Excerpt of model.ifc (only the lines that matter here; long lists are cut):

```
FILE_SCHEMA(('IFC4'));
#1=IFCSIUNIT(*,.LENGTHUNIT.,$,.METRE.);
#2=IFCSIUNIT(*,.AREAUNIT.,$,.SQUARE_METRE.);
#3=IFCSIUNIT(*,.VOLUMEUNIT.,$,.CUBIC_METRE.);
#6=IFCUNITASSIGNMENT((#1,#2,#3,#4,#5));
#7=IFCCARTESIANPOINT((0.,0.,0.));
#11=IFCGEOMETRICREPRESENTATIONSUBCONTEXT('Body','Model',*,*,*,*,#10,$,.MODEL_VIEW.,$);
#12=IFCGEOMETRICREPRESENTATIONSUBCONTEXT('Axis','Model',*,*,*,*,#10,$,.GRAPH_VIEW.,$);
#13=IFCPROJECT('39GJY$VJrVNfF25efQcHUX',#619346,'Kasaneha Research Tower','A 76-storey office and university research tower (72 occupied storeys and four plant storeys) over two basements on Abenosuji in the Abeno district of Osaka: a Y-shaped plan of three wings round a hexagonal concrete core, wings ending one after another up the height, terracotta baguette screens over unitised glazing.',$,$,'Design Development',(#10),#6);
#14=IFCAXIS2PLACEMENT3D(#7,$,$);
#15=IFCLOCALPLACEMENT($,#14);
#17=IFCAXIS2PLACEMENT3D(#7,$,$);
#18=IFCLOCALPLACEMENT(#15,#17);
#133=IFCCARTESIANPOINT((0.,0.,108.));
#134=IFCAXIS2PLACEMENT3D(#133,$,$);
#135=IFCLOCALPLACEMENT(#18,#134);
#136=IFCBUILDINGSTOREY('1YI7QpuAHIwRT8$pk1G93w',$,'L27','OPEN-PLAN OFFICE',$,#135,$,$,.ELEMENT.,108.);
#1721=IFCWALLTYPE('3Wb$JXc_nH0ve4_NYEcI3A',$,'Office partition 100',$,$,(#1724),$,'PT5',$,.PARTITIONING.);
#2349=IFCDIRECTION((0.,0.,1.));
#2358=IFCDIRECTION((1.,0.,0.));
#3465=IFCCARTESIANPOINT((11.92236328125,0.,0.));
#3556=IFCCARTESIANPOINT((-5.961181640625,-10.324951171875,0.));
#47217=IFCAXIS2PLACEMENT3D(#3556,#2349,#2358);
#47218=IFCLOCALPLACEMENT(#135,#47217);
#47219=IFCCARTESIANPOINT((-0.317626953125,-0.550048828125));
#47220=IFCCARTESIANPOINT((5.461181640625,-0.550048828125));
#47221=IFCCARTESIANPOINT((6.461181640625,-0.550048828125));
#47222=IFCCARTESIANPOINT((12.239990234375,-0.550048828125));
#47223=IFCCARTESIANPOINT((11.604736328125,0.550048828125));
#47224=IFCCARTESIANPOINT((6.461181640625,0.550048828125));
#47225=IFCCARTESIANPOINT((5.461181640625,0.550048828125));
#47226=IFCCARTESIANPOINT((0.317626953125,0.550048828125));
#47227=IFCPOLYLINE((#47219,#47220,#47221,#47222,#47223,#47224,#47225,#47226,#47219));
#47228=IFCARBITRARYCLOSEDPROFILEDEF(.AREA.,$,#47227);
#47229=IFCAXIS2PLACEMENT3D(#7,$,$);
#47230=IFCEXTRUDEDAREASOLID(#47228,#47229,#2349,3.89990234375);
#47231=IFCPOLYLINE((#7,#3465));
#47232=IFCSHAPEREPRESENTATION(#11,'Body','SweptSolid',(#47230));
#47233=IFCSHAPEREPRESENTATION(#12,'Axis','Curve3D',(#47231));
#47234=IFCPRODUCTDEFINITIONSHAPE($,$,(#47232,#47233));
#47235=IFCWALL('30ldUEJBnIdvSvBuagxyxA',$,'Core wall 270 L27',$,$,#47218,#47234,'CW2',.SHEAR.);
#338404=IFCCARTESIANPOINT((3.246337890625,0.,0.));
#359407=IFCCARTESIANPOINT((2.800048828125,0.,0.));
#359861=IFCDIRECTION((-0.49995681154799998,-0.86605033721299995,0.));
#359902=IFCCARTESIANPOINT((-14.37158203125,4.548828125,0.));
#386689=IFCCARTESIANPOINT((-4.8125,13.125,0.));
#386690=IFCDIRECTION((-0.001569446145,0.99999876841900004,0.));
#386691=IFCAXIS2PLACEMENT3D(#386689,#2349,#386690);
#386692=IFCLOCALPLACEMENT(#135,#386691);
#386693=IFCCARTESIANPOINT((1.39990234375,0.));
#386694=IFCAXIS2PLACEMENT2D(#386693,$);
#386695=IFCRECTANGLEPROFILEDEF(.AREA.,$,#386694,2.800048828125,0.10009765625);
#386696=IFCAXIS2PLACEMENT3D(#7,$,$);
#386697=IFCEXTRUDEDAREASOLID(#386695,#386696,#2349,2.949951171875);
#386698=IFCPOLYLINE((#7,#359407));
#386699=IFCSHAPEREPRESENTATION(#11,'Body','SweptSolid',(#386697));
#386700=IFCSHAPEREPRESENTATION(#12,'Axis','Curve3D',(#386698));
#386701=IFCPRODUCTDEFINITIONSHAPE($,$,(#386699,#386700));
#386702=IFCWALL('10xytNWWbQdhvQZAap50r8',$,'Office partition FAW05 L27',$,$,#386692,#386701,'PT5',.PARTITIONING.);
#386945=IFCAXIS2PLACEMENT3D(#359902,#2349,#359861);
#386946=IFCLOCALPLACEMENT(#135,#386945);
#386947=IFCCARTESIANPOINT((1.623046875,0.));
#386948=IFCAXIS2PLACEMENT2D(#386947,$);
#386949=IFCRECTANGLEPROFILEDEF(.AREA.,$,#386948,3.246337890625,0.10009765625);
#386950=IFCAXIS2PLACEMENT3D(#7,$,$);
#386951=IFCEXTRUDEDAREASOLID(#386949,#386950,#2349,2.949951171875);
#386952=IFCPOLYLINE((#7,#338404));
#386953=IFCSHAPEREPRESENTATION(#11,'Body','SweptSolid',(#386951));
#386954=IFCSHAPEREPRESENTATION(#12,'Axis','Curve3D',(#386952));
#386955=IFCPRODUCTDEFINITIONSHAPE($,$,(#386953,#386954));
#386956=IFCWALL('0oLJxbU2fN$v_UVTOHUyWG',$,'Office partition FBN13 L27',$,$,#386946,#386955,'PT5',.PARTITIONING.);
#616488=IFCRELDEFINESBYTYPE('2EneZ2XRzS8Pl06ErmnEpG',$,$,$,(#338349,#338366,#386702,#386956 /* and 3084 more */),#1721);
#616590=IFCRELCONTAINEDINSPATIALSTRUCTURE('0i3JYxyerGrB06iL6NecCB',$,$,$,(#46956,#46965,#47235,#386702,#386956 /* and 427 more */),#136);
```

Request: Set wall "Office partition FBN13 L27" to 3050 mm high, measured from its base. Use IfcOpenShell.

```python
import ifcopenshell
import ifcopenshell.geom
import ifcopenshell.util.representation
import ifcopenshell.util.shape
import ifcopenshell.util.unit

model = ifcopenshell.open("model.ifc")
unit_scale = ifcopenshell.util.unit.calculate_unit_scale(model)
settings = ifcopenshell.geom.settings()


def volume(element):
    """Net volume in cubic metres, openings subtracted."""
    shape = ifcopenshell.geom.create_shape(settings, element)
    return ifcopenshell.util.shape.get_volume(shape.geometry)


wall = model.by_guid("0oLJxbU2fN$v_UVTOHUyWG")
before = volume(wall)

body = ifcopenshell.util.representation.get_representation(wall, "Model", "Body")
solid = body.Items[0]
old_height = solid.Depth
solid.Depth = 3.05 / unit_scale
after = volume(wall)

print(f"height {old_height:g} -> {solid.Depth:g}, volume {before:.3f} -> {after:.3f} m3")

model.write("model_edited.ifc")
```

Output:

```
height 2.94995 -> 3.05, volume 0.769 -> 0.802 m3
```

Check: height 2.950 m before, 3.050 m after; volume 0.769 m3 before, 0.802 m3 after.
